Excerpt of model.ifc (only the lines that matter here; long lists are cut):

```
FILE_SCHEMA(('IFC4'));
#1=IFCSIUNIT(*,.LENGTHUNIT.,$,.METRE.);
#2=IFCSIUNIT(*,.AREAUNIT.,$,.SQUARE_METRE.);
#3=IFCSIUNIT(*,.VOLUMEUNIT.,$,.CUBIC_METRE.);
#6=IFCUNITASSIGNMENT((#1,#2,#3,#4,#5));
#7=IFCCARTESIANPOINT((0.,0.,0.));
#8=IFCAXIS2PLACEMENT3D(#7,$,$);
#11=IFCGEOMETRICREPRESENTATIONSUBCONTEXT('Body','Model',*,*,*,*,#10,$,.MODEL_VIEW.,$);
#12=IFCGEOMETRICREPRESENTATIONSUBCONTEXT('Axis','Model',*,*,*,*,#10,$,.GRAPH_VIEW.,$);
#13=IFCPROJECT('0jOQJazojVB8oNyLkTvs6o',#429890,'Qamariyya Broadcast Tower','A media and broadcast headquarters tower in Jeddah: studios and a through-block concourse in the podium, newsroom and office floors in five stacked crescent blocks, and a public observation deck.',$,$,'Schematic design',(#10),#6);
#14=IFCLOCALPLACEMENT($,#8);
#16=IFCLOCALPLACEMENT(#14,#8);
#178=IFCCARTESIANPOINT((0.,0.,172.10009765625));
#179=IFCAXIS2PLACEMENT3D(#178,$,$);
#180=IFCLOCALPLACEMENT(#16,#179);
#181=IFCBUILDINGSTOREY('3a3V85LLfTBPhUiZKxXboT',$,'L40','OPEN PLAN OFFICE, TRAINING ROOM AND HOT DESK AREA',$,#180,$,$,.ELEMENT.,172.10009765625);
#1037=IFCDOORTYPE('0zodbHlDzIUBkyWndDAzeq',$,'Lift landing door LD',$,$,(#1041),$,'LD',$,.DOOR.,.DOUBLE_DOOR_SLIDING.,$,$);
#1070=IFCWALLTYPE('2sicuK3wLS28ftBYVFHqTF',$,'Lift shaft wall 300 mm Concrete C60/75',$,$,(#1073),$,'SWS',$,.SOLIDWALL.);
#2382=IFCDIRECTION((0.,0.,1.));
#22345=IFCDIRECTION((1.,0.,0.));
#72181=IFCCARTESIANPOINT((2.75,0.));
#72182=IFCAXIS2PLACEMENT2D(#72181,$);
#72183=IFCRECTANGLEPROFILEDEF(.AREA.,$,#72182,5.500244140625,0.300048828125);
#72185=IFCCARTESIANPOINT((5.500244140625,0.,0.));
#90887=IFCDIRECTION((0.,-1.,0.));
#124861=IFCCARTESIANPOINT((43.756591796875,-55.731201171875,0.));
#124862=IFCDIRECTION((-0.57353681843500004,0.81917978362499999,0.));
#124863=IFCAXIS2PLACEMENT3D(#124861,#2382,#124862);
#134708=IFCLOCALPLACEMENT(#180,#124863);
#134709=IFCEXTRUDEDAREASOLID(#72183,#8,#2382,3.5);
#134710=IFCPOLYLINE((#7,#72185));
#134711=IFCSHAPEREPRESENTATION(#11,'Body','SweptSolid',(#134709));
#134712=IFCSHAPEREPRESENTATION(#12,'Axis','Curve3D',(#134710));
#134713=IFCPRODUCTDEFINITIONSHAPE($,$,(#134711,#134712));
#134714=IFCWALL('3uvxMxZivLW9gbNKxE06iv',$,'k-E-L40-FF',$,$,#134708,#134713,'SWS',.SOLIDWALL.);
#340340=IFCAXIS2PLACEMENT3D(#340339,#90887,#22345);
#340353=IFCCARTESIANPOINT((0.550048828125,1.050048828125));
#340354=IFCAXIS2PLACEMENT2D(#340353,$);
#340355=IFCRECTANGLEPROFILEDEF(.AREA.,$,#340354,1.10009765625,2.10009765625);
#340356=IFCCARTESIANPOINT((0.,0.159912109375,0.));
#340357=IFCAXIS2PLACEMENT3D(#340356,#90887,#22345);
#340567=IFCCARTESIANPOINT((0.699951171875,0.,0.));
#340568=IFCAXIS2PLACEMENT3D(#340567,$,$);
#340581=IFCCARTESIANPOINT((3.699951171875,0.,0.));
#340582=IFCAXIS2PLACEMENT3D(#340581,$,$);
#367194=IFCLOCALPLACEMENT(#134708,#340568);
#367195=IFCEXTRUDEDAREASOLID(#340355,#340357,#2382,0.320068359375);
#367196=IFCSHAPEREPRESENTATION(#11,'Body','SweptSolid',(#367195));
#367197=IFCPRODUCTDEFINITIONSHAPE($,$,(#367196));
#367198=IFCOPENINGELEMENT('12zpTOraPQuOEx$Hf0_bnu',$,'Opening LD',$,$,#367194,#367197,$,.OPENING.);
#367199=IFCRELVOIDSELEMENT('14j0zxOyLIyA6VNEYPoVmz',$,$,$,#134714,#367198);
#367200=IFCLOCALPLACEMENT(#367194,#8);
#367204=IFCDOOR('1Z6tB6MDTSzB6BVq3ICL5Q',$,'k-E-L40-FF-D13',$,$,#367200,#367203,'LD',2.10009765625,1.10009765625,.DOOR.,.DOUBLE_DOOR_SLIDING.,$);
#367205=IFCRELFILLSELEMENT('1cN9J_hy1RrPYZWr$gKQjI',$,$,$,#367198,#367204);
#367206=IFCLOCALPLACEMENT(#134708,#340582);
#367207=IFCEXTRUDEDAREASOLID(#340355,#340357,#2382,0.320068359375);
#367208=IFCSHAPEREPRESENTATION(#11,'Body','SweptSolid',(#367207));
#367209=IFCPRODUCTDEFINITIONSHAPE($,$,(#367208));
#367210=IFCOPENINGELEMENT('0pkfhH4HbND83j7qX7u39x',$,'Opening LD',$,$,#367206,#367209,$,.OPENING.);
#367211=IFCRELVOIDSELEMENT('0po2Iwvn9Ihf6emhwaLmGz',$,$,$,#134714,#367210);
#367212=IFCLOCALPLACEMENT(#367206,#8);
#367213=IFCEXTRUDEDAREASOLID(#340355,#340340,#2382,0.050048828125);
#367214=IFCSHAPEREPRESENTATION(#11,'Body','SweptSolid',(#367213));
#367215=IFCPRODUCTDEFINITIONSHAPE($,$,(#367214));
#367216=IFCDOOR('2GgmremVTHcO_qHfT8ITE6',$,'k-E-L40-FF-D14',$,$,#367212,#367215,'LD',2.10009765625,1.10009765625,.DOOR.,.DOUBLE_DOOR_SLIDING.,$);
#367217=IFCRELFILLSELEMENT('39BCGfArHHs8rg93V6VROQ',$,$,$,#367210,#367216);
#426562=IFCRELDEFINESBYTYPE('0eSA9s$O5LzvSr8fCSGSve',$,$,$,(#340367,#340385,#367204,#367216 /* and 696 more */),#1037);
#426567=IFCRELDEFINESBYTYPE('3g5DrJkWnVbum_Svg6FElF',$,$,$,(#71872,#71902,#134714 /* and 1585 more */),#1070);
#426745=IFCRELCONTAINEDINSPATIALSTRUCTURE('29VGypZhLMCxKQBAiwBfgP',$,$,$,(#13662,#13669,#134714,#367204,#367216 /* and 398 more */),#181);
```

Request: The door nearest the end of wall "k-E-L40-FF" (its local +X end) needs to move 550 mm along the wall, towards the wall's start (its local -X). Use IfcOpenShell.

```python
import ifcopenshell
import ifcopenshell.api.geometry
import ifcopenshell.util.placement

model = ifcopenshell.open("model.ifc")

door = model.by_id(367216)
opening = door.FillsVoids[0].RelatingOpeningElement
wall = opening.VoidsElements[0].RelatingBuildingElement

wall_matrix = ifcopenshell.util.placement.get_local_placement(wall.ObjectPlacement)
shift = wall_matrix[:3, 0] * -0.55
before = ifcopenshell.util.placement.get_local_placement(door.ObjectPlacement)[:3, 3].copy()

# The door is placed relative to its opening, so it follows when the opening moves.
matrix = ifcopenshell.util.placement.get_local_placement(opening.ObjectPlacement)
matrix[:3, 3] += shift
ifcopenshell.api.geometry.edit_object_placement(
    model, product=opening, matrix=matrix, is_si=False, should_transform_children=True
)

after = ifcopenshell.util.placement.get_local_placement(door.ObjectPlacement)[:3, 3]
print("door moved by", (after - before).round(3) + 0.0)

model.write("model-out.ifc")
```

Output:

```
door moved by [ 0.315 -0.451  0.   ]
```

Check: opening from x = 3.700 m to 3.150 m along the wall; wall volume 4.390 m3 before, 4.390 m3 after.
